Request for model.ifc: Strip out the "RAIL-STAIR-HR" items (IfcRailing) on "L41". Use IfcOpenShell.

First a look at what the model holds.

```python
import ifcopenshell
import ifcopenshell.util.element

model = ifcopenshell.open("model.ifc")
print(model.schema)
storey = next(s for s in model.by_type("IfcBuildingStorey") if s.Name == "L41")
railings = [e for e in ifcopenshell.util.element.get_decomposition(storey) if e.is_a("IfcRailing")]
seen = {}
for e in railings:
    element_type = ifcopenshell.util.element.get_type(e)
    name = element_type.Name if element_type not in (None, e) else None
    seen[name] = seen.get(name, 0) + 1
for name, count in sorted(seen.items(), key=str):
    print(count, "x", name)
```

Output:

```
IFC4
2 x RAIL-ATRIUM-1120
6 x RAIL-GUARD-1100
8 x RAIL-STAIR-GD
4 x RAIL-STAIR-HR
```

```python
import ifcopenshell
import ifcopenshell.api.root
import ifcopenshell.util.element

model = ifcopenshell.open("model.ifc")

storey = next(s for s in model.by_type("IfcBuildingStorey") if s.Name == "L41")
railings = [e for e in ifcopenshell.util.element.get_decomposition(storey) if e.is_a("IfcRailing")]
targets = [e for e in railings if (t := ifcopenshell.util.element.get_type(e)) not in (None, e) and t.Name == "RAIL-STAIR-HR"]

for e in targets:
    ifcopenshell.api.root.remove_product(model, product=e)
print(len(targets), "removed")

model.write("model_v2.ifc")
```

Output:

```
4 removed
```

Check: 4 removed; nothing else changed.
